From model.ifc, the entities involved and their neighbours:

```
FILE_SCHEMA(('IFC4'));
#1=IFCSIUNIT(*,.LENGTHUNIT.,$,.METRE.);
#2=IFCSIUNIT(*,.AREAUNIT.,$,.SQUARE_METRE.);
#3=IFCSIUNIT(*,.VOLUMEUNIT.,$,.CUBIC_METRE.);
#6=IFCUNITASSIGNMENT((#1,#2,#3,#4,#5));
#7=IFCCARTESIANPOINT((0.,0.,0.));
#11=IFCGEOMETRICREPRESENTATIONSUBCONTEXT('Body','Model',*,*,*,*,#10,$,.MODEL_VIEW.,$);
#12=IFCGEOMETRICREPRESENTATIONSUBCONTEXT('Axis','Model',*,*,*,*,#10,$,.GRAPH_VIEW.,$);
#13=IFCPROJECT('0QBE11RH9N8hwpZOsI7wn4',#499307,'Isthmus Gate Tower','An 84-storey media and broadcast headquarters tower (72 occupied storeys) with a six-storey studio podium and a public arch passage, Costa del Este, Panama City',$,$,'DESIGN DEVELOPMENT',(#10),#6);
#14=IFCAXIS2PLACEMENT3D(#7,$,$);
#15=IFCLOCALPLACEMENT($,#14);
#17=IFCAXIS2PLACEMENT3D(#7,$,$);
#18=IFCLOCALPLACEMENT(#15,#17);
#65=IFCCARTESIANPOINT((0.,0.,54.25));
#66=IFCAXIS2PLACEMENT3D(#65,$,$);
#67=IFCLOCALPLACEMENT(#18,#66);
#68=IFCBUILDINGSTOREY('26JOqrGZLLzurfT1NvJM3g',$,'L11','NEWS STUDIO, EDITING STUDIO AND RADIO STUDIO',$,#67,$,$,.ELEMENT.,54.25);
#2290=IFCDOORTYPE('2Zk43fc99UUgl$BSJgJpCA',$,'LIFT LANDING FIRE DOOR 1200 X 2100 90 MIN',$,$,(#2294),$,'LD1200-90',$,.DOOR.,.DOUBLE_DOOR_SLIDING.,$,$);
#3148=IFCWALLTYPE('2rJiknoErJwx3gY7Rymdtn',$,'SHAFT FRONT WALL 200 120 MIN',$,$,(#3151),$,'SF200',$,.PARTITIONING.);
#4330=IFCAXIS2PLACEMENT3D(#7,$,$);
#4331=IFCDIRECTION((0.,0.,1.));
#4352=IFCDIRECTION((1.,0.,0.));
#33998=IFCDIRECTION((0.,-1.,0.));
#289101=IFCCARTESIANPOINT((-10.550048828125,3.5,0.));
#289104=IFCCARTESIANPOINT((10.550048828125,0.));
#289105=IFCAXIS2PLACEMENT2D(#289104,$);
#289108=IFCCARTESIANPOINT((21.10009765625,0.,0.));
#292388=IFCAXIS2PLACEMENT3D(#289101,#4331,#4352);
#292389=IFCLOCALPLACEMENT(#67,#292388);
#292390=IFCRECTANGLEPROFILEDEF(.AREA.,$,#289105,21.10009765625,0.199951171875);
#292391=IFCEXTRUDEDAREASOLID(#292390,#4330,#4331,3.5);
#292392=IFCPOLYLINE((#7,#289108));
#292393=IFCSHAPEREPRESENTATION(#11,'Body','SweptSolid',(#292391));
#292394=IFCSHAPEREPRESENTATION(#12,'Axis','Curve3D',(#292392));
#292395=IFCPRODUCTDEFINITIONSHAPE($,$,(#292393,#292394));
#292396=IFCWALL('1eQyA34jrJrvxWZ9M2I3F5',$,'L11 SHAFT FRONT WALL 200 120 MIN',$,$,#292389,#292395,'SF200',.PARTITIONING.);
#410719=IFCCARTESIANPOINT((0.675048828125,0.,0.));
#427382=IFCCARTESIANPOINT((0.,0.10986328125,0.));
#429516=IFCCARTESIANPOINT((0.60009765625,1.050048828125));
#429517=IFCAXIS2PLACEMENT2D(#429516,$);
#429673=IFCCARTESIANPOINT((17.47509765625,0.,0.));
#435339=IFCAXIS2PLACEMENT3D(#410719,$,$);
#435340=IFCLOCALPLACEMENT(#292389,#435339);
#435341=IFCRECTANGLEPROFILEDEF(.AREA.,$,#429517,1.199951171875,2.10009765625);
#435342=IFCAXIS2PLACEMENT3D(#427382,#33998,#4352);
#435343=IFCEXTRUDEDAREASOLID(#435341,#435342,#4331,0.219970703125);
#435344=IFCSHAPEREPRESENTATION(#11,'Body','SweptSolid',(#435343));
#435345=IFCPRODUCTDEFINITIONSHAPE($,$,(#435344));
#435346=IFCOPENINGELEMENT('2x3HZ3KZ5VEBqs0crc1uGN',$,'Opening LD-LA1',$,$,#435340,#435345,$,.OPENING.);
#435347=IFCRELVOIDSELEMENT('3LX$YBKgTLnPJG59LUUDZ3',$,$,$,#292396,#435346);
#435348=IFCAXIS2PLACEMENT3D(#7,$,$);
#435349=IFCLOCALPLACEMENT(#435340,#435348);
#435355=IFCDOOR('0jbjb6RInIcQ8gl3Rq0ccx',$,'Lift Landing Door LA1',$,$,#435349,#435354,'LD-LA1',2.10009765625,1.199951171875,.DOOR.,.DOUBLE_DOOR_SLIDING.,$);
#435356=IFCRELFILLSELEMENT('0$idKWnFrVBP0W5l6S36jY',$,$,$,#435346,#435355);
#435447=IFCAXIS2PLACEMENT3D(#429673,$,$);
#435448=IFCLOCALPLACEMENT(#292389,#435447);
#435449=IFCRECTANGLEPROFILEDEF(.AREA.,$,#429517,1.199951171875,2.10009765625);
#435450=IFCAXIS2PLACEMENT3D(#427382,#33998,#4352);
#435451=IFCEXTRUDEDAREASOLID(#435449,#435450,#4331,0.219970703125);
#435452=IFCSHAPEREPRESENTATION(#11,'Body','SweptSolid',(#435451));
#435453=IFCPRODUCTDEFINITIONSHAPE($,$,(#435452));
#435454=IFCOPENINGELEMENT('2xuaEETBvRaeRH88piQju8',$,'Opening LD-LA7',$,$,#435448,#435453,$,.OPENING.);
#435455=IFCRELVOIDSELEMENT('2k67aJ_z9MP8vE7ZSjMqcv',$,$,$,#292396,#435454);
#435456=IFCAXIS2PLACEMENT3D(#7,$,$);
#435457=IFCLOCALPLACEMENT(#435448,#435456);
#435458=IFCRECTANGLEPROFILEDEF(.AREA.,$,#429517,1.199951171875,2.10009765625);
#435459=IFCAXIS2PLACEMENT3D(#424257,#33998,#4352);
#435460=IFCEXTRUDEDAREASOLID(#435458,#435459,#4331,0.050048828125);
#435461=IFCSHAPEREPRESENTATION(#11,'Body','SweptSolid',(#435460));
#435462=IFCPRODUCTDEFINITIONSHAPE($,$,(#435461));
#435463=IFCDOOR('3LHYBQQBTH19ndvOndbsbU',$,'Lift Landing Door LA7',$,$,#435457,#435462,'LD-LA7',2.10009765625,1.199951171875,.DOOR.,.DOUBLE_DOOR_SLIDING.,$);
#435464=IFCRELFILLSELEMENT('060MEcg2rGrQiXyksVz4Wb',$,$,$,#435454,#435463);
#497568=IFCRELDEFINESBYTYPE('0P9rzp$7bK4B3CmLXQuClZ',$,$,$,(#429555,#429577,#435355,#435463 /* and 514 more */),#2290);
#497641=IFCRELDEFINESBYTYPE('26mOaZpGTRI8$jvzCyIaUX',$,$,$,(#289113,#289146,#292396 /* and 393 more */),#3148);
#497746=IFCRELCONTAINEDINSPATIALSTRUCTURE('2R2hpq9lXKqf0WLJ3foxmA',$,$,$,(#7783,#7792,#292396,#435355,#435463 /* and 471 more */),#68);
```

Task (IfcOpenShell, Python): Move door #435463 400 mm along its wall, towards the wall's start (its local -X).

```python
import ifcopenshell
import ifcopenshell.api.geometry
import ifcopenshell.util.placement

model = ifcopenshell.open("model.ifc")

door = model.by_id(435463)
opening = door.FillsVoids[0].RelatingOpeningElement
wall = opening.VoidsElements[0].RelatingBuildingElement

wall_matrix = ifcopenshell.util.placement.get_local_placement(wall.ObjectPlacement)
shift = wall_matrix[:3, 0] * -0.4
before = ifcopenshell.util.placement.get_local_placement(door.ObjectPlacement)[:3, 3].copy()

# The door is placed relative to its opening, so it follows when the opening moves.
matrix = ifcopenshell.util.placement.get_local_placement(opening.ObjectPlacement)
matrix[:3, 3] += shift
ifcopenshell.api.geometry.edit_object_placement(
    model, product=opening, matrix=matrix, is_si=False, should_transform_children=True
)

after = ifcopenshell.util.placement.get_local_placement(door.ObjectPlacement)[:3, 3]
print("door moved by", (after - before).round(3) + 0.0)

model.write("model_updated.ifc")
```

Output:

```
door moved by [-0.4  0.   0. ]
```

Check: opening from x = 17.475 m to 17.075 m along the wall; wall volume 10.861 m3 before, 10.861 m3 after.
